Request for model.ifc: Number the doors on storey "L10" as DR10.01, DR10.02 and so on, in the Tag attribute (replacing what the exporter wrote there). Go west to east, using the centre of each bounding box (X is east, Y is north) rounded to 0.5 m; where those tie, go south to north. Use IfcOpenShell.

First a look at what the model holds.

```python
import ifcopenshell
import ifcopenshell.util.element
import ifcopenshell.util.placement

model = ifcopenshell.open("model.ifc")
print(model.schema)
storey = next(s for s in model.by_type("IfcBuildingStorey") if s.Name == "L10")
doors = [e for e in ifcopenshell.util.element.get_decomposition(storey) if e.is_a("IfcDoor")]
for e in sorted(doors, key=lambda e: e.id()):
    origin = ifcopenshell.util.placement.get_local_placement(e.ObjectPlacement)[:3, 3]
    print(e.id(), e.Tag, e.Name, origin.round(2) + 0.0, sep=" | ")
```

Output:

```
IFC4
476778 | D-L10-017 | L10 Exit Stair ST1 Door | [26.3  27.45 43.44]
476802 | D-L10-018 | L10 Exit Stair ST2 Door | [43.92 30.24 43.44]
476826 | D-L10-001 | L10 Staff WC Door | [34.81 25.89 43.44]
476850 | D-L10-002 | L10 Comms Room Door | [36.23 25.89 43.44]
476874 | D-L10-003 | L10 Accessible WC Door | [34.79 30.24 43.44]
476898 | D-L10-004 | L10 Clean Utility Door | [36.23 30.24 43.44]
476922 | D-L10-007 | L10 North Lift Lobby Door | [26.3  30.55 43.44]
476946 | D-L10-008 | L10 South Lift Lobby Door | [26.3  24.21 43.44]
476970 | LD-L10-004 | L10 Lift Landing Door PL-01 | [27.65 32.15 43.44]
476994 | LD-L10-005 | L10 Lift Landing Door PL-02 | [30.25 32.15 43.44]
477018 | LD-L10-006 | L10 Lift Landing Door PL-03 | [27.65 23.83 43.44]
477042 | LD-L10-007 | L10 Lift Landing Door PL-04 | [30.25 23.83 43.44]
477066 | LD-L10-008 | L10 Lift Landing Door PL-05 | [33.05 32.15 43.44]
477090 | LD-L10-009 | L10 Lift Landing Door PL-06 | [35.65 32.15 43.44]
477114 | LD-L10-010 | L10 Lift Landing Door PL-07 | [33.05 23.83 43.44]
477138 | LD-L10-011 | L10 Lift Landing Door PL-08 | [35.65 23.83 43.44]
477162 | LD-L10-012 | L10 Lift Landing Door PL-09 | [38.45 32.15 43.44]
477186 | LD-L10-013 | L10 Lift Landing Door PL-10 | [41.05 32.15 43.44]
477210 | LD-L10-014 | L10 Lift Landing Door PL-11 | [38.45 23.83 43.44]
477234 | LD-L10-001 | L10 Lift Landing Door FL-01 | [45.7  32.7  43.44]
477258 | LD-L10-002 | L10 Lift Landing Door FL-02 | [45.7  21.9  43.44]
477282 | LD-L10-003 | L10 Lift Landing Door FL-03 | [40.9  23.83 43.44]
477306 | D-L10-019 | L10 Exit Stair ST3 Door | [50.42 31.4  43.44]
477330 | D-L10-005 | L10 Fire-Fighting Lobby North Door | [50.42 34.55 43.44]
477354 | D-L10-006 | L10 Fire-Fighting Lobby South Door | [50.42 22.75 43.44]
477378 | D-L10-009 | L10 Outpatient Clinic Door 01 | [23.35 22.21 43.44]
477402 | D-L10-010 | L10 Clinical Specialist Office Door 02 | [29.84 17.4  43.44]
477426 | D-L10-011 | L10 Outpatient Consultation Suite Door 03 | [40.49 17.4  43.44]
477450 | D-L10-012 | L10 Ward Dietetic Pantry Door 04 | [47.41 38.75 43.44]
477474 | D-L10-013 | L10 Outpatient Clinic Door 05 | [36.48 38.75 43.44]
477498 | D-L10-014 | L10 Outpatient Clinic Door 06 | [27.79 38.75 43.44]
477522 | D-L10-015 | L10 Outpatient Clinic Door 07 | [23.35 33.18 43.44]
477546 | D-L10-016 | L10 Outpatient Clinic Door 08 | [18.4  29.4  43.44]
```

```python
import ifcopenshell
import ifcopenshell.geom
import ifcopenshell.util.element
import ifcopenshell.util.shape

model = ifcopenshell.open("model.ifc")
settings = ifcopenshell.geom.settings()
settings.set("use-world-coords", True)


def centre(element):
    shape = ifcopenshell.geom.create_shape(settings, element)
    return ifcopenshell.util.shape.get_bbox_centroid(shape.geometry)


storey = next(s for s in model.by_type("IfcBuildingStorey") if s.Name == "L10")
doors = [e for e in ifcopenshell.util.element.get_decomposition(storey) if e.is_a("IfcDoor")]

# Insertion points can sit at a corner or the storey origin, so sort by the geometry (in metres).
centres = {e: centre(e) for e in doors}
doors.sort(key=lambda e: (round(centres[e][0] / 0.5), centres[e][1]))

for i, e in enumerate(doors, start=1):
    number = f"DR10.{i:02d}"
    e.Tag = number
    print(e.id(), number)

model.write("model_edited.ifc")
```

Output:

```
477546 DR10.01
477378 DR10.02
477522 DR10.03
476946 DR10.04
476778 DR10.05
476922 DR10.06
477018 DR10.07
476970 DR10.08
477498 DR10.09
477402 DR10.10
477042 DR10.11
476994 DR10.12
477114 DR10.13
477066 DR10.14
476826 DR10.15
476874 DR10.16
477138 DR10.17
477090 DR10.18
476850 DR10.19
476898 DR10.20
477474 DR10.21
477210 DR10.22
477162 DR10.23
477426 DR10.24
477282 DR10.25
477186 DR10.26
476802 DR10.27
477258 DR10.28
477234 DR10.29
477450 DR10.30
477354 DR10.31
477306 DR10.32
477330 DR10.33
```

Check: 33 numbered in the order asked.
